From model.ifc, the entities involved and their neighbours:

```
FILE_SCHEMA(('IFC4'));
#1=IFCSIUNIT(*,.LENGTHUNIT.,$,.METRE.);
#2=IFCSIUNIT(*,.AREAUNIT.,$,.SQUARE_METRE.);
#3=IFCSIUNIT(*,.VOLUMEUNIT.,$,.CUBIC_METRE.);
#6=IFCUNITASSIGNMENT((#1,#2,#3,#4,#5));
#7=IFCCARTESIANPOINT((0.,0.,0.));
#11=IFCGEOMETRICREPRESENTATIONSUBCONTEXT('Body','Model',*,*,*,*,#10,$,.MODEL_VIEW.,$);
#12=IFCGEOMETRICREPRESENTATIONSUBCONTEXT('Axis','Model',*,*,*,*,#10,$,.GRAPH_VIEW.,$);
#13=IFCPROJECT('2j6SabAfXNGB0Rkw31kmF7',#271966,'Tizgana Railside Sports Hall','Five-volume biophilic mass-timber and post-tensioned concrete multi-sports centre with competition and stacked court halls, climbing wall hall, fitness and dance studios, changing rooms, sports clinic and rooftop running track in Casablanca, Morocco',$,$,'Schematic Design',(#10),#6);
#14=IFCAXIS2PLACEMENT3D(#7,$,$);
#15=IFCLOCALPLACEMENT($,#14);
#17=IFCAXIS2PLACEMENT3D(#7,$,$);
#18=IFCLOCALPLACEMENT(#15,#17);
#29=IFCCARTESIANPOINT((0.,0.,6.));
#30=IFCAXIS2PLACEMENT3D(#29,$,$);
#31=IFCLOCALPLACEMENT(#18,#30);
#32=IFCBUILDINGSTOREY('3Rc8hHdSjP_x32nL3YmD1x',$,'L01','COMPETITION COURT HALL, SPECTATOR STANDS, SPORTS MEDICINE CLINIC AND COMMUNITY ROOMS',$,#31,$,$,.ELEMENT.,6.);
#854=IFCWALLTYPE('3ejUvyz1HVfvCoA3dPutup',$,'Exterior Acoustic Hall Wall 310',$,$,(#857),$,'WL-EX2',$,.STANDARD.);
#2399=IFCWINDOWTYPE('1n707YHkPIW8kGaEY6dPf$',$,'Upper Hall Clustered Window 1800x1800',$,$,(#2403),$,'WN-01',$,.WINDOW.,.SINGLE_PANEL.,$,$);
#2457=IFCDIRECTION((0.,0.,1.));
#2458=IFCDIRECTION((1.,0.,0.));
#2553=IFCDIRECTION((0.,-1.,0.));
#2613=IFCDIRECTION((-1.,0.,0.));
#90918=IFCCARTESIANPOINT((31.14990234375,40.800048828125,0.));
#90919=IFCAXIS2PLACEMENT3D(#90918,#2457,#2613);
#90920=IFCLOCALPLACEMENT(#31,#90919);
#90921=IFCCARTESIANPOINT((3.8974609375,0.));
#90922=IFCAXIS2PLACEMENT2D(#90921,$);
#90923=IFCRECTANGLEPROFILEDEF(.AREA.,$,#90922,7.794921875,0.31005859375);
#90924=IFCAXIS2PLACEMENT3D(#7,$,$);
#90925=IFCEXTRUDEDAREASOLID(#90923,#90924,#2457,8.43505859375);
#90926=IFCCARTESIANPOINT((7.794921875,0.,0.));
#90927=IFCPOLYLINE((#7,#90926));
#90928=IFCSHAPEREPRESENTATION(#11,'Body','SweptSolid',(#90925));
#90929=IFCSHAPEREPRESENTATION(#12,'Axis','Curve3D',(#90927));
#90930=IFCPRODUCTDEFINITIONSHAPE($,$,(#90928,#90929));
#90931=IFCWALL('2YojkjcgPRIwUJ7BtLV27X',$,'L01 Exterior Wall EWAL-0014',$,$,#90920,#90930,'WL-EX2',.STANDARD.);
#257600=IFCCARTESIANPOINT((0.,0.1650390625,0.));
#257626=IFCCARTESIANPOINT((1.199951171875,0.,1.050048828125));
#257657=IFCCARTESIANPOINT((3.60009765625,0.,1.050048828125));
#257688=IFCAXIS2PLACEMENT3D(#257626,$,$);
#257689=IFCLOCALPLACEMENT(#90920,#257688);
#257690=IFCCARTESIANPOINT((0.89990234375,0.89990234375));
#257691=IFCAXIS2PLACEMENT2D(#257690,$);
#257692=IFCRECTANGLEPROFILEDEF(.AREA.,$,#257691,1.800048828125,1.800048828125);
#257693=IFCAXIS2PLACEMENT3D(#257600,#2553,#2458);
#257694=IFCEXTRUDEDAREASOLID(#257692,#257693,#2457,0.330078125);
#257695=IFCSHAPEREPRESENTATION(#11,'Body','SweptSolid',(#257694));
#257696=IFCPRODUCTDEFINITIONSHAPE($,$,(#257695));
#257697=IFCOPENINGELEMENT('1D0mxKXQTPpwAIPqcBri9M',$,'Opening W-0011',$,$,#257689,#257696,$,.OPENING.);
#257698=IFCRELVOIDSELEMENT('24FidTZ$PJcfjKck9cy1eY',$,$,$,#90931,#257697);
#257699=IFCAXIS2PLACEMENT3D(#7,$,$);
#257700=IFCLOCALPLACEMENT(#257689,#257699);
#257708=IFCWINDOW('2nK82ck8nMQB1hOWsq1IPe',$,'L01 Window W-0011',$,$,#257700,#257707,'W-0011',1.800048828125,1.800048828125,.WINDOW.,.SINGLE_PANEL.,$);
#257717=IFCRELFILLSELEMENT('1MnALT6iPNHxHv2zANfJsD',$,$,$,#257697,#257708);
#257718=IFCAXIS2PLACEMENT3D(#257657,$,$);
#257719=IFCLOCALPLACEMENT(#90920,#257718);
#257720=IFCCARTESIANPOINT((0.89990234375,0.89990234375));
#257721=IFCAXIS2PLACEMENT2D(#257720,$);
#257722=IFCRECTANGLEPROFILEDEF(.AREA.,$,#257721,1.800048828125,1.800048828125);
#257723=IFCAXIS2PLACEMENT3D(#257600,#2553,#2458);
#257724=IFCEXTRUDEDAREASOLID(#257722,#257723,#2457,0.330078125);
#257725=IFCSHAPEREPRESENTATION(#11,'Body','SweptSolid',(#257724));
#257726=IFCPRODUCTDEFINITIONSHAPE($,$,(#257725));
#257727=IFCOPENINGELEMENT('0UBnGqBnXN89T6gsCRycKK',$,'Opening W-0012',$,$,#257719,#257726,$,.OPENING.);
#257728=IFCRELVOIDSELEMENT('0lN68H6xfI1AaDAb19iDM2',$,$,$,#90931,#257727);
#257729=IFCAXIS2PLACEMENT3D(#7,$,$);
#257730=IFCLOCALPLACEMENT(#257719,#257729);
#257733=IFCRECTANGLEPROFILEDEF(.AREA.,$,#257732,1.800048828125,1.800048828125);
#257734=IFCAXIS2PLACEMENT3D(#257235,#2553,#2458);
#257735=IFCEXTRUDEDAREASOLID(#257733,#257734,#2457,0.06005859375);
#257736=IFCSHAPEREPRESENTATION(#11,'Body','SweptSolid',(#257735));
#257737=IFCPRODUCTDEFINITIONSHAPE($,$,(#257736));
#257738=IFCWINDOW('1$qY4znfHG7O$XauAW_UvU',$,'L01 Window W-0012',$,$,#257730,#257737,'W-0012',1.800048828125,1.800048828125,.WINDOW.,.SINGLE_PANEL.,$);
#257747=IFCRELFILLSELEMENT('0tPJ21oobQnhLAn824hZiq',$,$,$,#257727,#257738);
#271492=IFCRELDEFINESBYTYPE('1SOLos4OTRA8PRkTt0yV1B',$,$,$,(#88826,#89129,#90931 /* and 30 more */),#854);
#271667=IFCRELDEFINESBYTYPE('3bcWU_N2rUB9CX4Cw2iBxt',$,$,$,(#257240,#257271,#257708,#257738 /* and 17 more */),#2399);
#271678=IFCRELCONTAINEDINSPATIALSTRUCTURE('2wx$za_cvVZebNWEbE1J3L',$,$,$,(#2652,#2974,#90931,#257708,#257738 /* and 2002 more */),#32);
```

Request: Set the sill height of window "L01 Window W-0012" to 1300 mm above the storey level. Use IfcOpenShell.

```python
import numpy as np
import ifcopenshell
import ifcopenshell.api.geometry
import ifcopenshell.geom
import ifcopenshell.util.element
import ifcopenshell.util.placement
import ifcopenshell.util.shape
import ifcopenshell.util.unit

model = ifcopenshell.open("model.ifc")
unit_scale = ifcopenshell.util.unit.calculate_unit_scale(model)

window = model.by_guid("1$qY4znfHG7O$XauAW_UvU")
opening = window.FillsVoids[0].RelatingOpeningElement
storey = ifcopenshell.util.element.get_container(window, ifc_class="IfcBuildingStorey")
level = ifcopenshell.util.placement.get_local_placement(storey.ObjectPlacement)[2, 3]

# The opening's origin need not be at the sill, so measure its lowest point.
shape = ifcopenshell.geom.create_shape(ifcopenshell.geom.settings(), opening)
bottom = ifcopenshell.util.shape.get_shape_bottom_elevation(shape, shape.geometry) / unit_scale
dz = level + 1.3 / unit_scale - bottom

shift = np.array([0.0, 0.0, dz])
# The window is placed relative to its opening, so it follows when the opening moves.
matrix = ifcopenshell.util.placement.get_local_placement(opening.ObjectPlacement)
matrix[:3, 3] += shift
ifcopenshell.api.geometry.edit_object_placement(
    model, product=opening, matrix=matrix, is_si=False, should_transform_children=True
)

print(f"moved by {dz * unit_scale:+.3f} m")

model.write("model-out.ifc")
```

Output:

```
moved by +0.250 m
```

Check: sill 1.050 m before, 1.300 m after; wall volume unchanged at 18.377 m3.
